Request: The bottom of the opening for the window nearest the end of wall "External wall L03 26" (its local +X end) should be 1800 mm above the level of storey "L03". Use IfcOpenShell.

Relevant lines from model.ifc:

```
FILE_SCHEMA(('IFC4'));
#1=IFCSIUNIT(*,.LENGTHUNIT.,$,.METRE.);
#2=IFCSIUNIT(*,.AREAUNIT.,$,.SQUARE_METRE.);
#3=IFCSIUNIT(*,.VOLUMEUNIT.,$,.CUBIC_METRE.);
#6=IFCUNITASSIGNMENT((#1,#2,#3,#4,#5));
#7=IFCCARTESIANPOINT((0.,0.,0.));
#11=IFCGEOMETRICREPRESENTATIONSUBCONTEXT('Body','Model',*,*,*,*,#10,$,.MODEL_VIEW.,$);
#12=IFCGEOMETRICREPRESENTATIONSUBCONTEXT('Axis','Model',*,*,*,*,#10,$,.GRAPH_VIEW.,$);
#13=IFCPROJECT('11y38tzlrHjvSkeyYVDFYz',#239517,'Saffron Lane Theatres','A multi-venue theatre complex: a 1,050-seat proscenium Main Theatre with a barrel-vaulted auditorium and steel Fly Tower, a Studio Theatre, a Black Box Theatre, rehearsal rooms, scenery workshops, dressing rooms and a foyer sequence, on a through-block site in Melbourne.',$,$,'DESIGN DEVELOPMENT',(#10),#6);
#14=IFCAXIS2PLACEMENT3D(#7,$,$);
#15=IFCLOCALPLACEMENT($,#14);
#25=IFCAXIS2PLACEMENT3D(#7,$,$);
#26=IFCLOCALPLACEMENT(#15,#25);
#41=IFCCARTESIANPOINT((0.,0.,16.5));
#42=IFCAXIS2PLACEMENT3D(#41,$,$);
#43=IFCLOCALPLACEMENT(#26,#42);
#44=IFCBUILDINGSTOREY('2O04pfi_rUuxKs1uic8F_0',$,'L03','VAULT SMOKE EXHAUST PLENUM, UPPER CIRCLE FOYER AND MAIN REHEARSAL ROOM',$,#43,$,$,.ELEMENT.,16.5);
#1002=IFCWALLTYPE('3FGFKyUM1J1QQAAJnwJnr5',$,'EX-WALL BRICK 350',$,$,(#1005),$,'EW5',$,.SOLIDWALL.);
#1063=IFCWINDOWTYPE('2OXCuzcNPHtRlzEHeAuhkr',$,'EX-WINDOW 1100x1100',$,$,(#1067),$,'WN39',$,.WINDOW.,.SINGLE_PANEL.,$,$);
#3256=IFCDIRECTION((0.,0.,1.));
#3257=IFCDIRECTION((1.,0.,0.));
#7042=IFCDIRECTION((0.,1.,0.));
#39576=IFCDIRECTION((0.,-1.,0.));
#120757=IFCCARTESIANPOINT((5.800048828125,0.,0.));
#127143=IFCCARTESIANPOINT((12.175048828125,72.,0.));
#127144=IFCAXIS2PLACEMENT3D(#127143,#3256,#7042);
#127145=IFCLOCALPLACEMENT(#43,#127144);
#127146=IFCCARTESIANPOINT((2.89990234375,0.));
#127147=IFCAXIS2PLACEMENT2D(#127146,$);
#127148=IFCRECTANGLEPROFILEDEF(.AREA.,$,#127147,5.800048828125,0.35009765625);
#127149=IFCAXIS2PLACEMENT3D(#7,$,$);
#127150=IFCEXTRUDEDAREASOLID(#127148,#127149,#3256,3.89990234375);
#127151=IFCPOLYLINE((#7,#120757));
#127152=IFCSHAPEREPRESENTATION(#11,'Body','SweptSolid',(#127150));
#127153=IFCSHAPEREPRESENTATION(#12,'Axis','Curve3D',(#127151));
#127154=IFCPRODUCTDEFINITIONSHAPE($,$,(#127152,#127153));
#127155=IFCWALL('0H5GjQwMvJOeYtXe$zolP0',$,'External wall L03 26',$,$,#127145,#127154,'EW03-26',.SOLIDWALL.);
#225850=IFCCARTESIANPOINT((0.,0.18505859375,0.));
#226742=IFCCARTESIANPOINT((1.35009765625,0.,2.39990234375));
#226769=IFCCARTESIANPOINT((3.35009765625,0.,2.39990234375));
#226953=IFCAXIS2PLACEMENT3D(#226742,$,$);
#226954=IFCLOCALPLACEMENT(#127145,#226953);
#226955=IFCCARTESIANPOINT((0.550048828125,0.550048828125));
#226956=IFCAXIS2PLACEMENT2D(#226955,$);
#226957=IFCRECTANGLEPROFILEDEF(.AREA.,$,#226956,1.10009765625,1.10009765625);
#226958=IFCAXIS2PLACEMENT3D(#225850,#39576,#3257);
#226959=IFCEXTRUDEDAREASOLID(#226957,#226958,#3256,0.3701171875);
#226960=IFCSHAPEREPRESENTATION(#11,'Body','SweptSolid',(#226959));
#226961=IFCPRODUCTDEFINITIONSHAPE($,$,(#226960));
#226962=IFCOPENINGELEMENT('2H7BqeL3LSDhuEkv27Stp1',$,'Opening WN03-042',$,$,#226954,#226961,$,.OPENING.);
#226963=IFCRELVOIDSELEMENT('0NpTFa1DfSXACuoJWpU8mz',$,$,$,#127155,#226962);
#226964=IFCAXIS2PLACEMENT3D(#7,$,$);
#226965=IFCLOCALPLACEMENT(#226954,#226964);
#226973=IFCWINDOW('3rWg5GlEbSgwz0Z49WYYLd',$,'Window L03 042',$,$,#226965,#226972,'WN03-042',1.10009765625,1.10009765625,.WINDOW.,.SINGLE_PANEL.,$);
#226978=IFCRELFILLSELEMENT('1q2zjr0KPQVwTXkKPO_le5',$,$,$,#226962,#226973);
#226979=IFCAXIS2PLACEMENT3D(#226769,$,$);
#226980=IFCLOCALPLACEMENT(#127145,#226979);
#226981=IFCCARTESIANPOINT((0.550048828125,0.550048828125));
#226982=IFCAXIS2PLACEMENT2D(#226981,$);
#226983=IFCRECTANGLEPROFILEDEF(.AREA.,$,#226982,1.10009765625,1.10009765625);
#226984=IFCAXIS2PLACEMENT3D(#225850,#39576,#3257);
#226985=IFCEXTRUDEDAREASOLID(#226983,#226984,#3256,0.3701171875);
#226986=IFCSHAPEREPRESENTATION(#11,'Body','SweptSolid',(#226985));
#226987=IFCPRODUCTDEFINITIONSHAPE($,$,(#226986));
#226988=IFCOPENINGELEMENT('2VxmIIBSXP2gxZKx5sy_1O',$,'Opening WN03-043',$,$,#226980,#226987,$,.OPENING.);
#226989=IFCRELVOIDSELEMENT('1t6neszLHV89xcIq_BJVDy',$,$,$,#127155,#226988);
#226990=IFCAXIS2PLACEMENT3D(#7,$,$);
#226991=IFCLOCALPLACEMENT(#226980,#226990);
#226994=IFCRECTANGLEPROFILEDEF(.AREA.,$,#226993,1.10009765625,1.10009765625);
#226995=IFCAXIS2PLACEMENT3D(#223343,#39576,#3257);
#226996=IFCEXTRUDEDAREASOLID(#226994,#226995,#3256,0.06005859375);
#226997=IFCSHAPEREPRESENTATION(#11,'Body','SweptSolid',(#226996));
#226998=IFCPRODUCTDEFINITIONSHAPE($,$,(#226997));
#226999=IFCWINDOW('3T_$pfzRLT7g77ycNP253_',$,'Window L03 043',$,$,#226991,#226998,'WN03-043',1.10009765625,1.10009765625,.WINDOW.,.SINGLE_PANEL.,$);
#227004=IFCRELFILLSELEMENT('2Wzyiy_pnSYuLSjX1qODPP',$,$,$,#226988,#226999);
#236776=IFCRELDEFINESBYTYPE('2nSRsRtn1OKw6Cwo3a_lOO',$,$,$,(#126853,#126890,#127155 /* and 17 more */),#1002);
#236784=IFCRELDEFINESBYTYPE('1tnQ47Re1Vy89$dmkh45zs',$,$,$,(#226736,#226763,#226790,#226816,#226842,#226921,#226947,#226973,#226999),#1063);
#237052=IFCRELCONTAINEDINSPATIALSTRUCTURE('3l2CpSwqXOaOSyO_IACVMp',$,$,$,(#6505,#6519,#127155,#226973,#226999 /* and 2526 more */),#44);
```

```python
import numpy as np
import ifcopenshell
import ifcopenshell.api.geometry
import ifcopenshell.geom
import ifcopenshell.util.element
import ifcopenshell.util.placement
import ifcopenshell.util.shape
import ifcopenshell.util.unit

model = ifcopenshell.open("model.ifc")
unit_scale = ifcopenshell.util.unit.calculate_unit_scale(model)

window = model.by_guid("3T_$pfzRLT7g77ycNP253_")
opening = window.FillsVoids[0].RelatingOpeningElement
storey = ifcopenshell.util.element.get_container(window, ifc_class="IfcBuildingStorey")
level = ifcopenshell.util.placement.get_local_placement(storey.ObjectPlacement)[2, 3]

# The opening's origin need not be at the sill, so measure its lowest point.
shape = ifcopenshell.geom.create_shape(ifcopenshell.geom.settings(), opening)
bottom = ifcopenshell.util.shape.get_shape_bottom_elevation(shape, shape.geometry) / unit_scale
dz = level + 1.8 - bottom

shift = np.array([0.0, 0.0, dz])
# The window is placed relative to its opening, so it follows when the opening moves.
matrix = ifcopenshell.util.placement.get_local_placement(opening.ObjectPlacement)
matrix[:3, 3] += shift
ifcopenshell.api.geometry.edit_object_placement(
    model, product=opening, matrix=matrix, is_si=False, should_transform_children=True
)

print(f"moved by {dz * unit_scale:+.3f} m")

model.write("model_rev.ifc")
```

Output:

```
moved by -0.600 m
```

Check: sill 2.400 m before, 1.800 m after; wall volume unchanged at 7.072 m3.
